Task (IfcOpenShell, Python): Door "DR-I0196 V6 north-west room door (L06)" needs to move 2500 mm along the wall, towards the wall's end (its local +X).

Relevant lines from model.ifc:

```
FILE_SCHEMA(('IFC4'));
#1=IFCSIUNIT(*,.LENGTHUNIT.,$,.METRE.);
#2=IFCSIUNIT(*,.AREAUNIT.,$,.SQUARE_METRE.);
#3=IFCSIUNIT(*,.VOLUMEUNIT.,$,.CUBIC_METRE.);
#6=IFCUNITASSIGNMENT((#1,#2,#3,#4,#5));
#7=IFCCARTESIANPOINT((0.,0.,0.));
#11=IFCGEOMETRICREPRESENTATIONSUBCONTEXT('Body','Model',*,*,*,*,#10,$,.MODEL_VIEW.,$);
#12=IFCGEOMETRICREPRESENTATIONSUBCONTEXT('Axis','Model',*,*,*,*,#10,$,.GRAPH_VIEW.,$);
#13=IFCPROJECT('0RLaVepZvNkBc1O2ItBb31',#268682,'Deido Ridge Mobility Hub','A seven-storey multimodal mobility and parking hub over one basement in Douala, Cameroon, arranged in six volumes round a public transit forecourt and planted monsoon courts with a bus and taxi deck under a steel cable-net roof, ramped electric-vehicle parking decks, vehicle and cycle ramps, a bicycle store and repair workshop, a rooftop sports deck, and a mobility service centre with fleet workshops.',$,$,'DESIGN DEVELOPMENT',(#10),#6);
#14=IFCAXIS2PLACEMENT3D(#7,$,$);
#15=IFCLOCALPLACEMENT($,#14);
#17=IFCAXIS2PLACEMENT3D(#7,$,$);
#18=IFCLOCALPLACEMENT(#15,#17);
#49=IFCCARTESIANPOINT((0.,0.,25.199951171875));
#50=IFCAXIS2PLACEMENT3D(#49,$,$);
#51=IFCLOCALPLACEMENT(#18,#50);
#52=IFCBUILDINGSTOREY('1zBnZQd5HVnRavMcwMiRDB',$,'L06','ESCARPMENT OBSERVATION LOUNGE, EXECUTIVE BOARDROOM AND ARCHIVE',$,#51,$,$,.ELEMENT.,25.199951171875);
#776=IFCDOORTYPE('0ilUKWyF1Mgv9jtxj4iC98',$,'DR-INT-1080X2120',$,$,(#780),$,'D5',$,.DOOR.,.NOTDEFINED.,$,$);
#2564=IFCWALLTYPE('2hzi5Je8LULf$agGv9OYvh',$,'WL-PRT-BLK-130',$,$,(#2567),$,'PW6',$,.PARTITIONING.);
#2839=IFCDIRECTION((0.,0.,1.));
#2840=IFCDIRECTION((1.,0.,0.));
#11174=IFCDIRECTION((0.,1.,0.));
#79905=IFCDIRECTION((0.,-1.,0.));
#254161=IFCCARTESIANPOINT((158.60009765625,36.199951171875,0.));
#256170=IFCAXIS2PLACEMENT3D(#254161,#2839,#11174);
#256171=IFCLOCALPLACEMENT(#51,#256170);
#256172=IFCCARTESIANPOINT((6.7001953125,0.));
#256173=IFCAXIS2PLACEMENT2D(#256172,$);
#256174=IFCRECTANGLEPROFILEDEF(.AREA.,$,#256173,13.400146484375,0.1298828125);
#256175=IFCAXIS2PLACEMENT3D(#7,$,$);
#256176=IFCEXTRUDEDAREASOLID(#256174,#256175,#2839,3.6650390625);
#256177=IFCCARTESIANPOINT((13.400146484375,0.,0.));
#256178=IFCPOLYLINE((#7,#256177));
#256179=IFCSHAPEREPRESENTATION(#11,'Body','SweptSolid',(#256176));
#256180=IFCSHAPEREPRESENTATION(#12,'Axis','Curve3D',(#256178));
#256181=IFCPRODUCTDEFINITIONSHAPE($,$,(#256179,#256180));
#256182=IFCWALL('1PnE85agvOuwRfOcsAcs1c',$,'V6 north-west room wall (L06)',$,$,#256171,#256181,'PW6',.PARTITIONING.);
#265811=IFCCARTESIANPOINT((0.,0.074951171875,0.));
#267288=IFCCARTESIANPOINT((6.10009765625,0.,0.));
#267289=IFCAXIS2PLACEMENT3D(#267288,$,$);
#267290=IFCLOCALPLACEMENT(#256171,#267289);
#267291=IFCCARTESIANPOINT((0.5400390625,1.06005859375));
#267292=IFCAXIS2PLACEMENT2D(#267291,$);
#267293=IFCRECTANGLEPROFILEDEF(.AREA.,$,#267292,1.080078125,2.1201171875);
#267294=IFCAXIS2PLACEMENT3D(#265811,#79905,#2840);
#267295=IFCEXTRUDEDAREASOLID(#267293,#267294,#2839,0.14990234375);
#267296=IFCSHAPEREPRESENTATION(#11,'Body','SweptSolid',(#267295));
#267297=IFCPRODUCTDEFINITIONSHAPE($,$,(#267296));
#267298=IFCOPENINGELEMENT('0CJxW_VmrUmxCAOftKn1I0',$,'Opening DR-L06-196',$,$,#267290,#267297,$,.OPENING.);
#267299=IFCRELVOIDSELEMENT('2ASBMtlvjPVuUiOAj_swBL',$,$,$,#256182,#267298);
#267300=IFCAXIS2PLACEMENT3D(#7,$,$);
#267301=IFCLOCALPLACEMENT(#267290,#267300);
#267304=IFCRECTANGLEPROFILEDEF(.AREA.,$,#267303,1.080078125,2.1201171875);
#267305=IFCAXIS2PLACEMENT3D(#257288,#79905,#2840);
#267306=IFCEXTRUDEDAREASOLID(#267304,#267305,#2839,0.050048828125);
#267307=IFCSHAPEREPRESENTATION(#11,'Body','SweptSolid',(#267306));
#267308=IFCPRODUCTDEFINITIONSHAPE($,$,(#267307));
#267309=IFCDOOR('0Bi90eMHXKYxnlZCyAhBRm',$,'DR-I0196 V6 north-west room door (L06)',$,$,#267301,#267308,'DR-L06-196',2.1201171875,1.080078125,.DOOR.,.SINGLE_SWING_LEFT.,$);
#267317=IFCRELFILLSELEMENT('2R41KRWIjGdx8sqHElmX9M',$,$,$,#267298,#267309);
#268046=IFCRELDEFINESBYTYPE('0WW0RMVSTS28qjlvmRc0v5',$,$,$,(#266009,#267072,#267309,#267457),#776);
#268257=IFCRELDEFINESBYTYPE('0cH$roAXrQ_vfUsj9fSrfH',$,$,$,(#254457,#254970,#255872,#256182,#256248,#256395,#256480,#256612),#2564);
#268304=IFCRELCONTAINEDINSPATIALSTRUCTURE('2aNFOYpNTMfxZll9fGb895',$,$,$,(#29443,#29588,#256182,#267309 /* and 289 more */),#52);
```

```python
import ifcopenshell
import ifcopenshell.api.geometry
import ifcopenshell.util.placement
import ifcopenshell.util.unit

model = ifcopenshell.open("model.ifc")
unit_scale = ifcopenshell.util.unit.calculate_unit_scale(model)

door = model.by_guid("0Bi90eMHXKYxnlZCyAhBRm")
opening = door.FillsVoids[0].RelatingOpeningElement
wall = opening.VoidsElements[0].RelatingBuildingElement

wall_matrix = ifcopenshell.util.placement.get_local_placement(wall.ObjectPlacement)
shift = wall_matrix[:3, 0] * 2.5 / unit_scale
before = ifcopenshell.util.placement.get_local_placement(door.ObjectPlacement)[:3, 3].copy()

# The door is placed relative to its opening, so it follows when the opening moves.
matrix = ifcopenshell.util.placement.get_local_placement(opening.ObjectPlacement)
matrix[:3, 3] += shift
ifcopenshell.api.geometry.edit_object_placement(
    model, product=opening, matrix=matrix, is_si=False, should_transform_children=True
)

after = ifcopenshell.util.placement.get_local_placement(door.ObjectPlacement)[:3, 3]
print("door moved by", (after - before).round(3) + 0.0)

model.write("model_v2.ifc")
```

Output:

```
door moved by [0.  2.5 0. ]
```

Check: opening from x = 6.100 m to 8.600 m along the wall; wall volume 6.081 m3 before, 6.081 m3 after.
